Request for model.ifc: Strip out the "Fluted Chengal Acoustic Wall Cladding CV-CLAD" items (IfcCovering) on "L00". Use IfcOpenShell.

First a look at what the model holds.

```python
import ifcopenshell
import ifcopenshell.util.element

model = ifcopenshell.open("model.ifc")
print(model.schema)
storey = next(s for s in model.by_type("IfcBuildingStorey") if s.Name == "L00")
coverings = [e for e in ifcopenshell.util.element.get_decomposition(storey) if e.is_a("IfcCovering")]
seen = {}
for e in coverings:
    element_type = ifcopenshell.util.element.get_type(e)
    name = element_type.Name if element_type not in (None, e) else None
    seen[name] = seen.get(name, 0) + 1
for name, count in sorted(seen.items(), key=str):
    print(count, "x", name)
```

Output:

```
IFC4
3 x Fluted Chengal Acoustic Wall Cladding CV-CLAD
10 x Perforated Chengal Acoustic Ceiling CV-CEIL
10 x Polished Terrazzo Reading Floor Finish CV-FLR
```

```python
import ifcopenshell
import ifcopenshell.api.root
import ifcopenshell.util.element

model = ifcopenshell.open("model.ifc")

storey = next(s for s in model.by_type("IfcBuildingStorey") if s.Name == "L00")
coverings = [e for e in ifcopenshell.util.element.get_decomposition(storey) if e.is_a("IfcCovering")]
targets = [e for e in coverings if (t := ifcopenshell.util.element.get_type(e)) not in (None, e) and t.Name == "Fluted Chengal Acoustic Wall Cladding CV-CLAD"]

for e in targets:
    ifcopenshell.api.root.remove_product(model, product=e)
print(len(targets), "removed")

model.write("model_edited.ifc")
```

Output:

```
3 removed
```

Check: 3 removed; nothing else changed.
